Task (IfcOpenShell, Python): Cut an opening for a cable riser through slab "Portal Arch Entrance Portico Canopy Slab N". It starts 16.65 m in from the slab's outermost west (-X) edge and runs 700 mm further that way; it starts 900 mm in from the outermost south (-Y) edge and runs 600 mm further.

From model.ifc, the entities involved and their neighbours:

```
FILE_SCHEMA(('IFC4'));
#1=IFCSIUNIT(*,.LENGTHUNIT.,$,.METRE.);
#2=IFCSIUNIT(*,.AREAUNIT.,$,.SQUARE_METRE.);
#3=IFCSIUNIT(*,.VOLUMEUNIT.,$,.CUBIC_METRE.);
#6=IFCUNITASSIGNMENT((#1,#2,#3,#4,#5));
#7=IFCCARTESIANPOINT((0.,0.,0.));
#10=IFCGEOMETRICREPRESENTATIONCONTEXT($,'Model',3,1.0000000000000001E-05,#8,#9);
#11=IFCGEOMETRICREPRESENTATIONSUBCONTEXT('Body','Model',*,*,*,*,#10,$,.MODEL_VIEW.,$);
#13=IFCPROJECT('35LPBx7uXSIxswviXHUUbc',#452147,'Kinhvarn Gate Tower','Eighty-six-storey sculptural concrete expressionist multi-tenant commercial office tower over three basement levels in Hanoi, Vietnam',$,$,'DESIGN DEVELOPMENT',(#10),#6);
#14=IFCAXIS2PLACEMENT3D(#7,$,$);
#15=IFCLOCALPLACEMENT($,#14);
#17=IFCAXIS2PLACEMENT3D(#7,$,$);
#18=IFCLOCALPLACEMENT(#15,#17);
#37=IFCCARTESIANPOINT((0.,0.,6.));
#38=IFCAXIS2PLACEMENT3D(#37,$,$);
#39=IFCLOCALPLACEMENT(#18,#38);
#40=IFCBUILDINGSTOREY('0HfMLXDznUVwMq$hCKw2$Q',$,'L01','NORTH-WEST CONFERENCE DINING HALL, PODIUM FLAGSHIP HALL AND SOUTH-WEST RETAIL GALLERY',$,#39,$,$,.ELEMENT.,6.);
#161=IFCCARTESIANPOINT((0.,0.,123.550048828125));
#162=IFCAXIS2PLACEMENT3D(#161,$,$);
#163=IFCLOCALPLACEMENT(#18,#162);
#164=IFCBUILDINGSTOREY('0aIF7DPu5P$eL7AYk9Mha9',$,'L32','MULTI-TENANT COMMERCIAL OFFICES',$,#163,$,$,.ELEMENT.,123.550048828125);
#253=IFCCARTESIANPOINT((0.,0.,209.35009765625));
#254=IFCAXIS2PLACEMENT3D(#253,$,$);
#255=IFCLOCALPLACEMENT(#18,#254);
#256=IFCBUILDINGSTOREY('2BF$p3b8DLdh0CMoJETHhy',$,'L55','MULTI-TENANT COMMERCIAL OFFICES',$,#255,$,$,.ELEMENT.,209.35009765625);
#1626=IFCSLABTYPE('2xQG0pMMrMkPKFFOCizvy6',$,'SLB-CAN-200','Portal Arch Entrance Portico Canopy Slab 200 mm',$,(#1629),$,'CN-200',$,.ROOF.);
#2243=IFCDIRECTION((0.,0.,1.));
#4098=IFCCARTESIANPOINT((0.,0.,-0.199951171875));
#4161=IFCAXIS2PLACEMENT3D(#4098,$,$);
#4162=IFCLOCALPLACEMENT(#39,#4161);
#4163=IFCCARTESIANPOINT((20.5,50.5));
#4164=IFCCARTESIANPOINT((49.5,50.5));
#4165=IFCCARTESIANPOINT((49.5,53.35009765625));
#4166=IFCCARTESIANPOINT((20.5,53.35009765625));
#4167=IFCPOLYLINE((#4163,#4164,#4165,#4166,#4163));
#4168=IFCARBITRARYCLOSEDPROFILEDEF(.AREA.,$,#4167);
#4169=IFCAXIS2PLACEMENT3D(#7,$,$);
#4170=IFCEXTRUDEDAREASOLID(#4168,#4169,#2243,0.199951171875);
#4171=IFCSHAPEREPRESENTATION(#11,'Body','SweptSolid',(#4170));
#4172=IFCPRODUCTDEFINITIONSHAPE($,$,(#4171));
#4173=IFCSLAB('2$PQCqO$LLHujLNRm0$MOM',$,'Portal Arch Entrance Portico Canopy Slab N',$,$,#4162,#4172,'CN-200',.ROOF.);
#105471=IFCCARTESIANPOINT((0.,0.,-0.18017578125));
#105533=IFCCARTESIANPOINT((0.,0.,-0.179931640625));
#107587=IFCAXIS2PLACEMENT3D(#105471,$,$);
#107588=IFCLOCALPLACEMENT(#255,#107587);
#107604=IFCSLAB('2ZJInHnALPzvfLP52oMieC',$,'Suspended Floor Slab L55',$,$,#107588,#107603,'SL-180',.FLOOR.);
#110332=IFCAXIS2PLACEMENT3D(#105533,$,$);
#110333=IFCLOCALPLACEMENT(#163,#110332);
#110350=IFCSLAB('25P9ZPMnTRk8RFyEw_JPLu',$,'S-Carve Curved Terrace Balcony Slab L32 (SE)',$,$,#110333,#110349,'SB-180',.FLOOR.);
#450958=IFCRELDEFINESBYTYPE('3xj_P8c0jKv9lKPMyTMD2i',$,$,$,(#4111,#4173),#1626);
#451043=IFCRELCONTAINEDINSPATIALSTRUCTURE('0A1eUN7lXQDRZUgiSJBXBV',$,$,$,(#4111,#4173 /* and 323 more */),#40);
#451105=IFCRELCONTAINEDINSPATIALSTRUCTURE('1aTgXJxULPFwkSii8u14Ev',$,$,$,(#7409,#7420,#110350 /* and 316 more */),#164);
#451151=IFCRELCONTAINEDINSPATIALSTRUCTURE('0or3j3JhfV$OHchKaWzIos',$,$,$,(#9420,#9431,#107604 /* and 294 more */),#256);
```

```python
import numpy as np
import ifcopenshell
import ifcopenshell.api.feature
import ifcopenshell.api.geometry
import ifcopenshell.api.root
import ifcopenshell.geom
import ifcopenshell.util.placement
import ifcopenshell.util.representation
import ifcopenshell.util.shape
import ifcopenshell.util.unit

model = ifcopenshell.open("model.ifc")
unit_scale = ifcopenshell.util.unit.calculate_unit_scale(model)
settings = ifcopenshell.geom.settings()


def volume(element):
    """Net volume in cubic metres, openings subtracted."""
    shape = ifcopenshell.geom.create_shape(settings, element)
    return ifcopenshell.util.shape.get_volume(shape.geometry)


slab = model.by_guid("2$PQCqO$LLHujLNRm0$MOM")
before = volume(slab)

# Extent in the slab's own axes, in metres. The edges named are its -X and -Y sides.
slab_shape = ifcopenshell.geom.create_shape(settings, slab)
vertices = ifcopenshell.util.shape.get_vertices(slab_shape.geometry)
x_min, y_min, bottom = vertices.min(axis=0)
top = vertices[:, 2].max()

opening = ifcopenshell.api.root.create_entity(model, ifc_class="IfcOpeningElement", name="Cable riser opening", predefined_type="OPENING")
context = ifcopenshell.util.representation.get_context(model, "Model", "Body", "MODEL_VIEW")
width, depth = 0.7, 0.6
outline = [(0.0, 0.0), (width, 0.0), (width, depth), (0.0, depth), (0.0, 0.0)]
# Overshoot both faces by 50 mm so the cut is clean.
shape = ifcopenshell.api.geometry.add_slab_representation(
    model, context=context, depth=top - bottom + 0.1, polyline=outline
)
ifcopenshell.api.geometry.assign_representation(model, product=opening, representation=shape)

matrix = ifcopenshell.util.placement.get_local_placement(slab.ObjectPlacement)
matrix[:, 3] = matrix @ np.append(np.array([x_min + 16.65, y_min + 0.9, bottom - 0.05]) / unit_scale, 1.0)
ifcopenshell.api.geometry.edit_object_placement(model, product=opening, matrix=matrix, is_si=False)
ifcopenshell.api.feature.add_feature(model, feature=opening, element=slab)

after = volume(slab)

print(f"slab volume {before:.3f} -> {after:.3f} m3")

model.write("model-out.ifc")
```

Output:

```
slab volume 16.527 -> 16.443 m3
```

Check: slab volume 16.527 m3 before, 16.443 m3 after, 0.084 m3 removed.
